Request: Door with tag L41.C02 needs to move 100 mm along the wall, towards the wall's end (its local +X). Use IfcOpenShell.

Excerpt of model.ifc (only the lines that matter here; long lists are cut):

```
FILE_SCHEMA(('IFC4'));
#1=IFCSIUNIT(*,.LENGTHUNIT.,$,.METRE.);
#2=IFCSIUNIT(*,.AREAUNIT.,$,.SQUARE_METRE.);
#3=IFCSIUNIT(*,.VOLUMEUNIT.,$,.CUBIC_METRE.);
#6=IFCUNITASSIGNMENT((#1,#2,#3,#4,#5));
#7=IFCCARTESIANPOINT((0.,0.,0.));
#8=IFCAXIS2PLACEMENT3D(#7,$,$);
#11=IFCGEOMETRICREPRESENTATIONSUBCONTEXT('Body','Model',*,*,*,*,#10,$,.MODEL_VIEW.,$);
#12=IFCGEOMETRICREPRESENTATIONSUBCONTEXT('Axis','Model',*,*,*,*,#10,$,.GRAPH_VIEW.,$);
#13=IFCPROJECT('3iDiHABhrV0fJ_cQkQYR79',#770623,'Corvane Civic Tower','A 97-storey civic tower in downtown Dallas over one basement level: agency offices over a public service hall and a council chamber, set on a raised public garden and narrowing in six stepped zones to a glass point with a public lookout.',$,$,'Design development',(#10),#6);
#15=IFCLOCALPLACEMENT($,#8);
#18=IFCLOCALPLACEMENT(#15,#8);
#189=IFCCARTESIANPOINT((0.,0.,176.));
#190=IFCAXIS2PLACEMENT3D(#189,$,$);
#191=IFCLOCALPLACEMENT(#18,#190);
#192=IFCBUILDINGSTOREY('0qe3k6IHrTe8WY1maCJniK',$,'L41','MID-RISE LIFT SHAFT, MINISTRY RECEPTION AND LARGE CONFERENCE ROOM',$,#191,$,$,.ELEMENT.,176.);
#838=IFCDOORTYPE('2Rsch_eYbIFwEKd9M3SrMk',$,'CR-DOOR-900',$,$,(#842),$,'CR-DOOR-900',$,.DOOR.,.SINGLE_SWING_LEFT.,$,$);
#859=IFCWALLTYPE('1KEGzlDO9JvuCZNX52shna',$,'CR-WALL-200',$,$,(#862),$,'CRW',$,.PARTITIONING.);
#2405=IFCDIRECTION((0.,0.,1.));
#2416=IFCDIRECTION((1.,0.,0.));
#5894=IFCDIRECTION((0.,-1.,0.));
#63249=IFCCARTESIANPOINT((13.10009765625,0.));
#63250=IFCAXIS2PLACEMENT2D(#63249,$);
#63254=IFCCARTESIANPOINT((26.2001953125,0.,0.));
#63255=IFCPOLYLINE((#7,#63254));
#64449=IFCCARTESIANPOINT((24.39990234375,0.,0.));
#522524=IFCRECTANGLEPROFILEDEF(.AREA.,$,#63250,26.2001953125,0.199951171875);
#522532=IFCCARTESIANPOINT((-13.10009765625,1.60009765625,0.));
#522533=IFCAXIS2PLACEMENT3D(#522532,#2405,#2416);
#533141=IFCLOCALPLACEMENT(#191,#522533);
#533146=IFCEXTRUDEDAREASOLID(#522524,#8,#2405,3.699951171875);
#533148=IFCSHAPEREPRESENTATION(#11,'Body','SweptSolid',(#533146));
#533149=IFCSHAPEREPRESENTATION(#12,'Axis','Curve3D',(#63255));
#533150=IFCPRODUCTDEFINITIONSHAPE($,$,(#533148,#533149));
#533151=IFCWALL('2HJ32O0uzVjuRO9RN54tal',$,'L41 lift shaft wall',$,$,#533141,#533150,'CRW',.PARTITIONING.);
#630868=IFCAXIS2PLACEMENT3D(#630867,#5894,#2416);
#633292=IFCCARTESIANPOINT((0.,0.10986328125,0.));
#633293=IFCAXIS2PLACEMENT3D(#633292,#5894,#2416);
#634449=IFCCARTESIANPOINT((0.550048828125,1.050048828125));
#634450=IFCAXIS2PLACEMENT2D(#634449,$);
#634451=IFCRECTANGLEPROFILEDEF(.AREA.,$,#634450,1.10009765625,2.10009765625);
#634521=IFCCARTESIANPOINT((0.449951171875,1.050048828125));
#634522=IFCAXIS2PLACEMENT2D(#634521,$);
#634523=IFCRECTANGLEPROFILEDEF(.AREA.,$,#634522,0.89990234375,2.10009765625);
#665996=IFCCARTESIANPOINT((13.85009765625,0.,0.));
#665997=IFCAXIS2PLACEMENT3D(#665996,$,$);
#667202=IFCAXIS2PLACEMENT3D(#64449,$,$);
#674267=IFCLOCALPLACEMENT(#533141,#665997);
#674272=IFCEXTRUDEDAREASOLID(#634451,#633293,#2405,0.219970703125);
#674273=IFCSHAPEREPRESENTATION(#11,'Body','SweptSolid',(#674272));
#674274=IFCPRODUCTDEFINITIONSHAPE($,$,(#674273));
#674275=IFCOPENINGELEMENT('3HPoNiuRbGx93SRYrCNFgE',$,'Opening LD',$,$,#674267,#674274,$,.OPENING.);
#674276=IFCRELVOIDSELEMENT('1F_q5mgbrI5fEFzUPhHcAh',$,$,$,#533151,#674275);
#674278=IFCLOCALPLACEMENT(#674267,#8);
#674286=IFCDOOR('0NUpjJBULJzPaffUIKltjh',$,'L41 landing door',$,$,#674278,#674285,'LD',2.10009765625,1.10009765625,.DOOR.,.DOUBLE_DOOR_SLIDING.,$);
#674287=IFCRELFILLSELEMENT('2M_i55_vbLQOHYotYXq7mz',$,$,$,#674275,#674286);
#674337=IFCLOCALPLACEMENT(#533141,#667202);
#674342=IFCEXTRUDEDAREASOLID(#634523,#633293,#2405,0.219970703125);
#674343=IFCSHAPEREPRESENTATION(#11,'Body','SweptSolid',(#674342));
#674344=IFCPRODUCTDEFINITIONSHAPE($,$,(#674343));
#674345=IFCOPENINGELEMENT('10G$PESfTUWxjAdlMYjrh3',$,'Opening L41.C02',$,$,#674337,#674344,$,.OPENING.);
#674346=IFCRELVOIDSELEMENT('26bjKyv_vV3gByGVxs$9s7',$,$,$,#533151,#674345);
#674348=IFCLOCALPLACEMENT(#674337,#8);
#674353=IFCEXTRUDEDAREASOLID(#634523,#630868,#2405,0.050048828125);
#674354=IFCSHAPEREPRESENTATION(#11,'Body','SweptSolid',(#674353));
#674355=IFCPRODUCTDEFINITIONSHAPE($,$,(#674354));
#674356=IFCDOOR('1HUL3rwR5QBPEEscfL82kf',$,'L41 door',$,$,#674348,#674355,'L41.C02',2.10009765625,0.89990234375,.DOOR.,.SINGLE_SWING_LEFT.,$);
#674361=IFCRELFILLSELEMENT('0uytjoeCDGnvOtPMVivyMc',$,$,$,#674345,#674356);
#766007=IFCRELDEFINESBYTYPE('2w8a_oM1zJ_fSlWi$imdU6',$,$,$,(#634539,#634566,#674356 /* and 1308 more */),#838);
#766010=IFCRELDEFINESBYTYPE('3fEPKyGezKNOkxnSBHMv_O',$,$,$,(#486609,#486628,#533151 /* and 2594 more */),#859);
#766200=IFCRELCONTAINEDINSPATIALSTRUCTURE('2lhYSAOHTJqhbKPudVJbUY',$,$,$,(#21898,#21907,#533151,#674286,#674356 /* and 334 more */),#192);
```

```python
import ifcopenshell
import ifcopenshell.api.geometry
import ifcopenshell.util.placement

model = ifcopenshell.open("model.ifc")

door = model.by_id(674356)
opening = door.FillsVoids[0].RelatingOpeningElement
wall = opening.VoidsElements[0].RelatingBuildingElement

wall_matrix = ifcopenshell.util.placement.get_local_placement(wall.ObjectPlacement)
shift = wall_matrix[:3, 0] * 0.1
before = ifcopenshell.util.placement.get_local_placement(door.ObjectPlacement)[:3, 3].copy()

# The door is placed relative to its opening, so it follows when the opening moves.
matrix = ifcopenshell.util.placement.get_local_placement(opening.ObjectPlacement)
matrix[:3, 3] += shift
ifcopenshell.api.geometry.edit_object_placement(
    model, product=opening, matrix=matrix, is_si=False, should_transform_children=True
)

after = ifcopenshell.util.placement.get_local_placement(door.ObjectPlacement)[:3, 3]
print("door moved by", (after - before).round(3) + 0.0)

model.write("model_v2.ifc")
```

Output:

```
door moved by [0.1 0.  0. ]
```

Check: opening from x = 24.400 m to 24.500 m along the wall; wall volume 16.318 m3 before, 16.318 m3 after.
